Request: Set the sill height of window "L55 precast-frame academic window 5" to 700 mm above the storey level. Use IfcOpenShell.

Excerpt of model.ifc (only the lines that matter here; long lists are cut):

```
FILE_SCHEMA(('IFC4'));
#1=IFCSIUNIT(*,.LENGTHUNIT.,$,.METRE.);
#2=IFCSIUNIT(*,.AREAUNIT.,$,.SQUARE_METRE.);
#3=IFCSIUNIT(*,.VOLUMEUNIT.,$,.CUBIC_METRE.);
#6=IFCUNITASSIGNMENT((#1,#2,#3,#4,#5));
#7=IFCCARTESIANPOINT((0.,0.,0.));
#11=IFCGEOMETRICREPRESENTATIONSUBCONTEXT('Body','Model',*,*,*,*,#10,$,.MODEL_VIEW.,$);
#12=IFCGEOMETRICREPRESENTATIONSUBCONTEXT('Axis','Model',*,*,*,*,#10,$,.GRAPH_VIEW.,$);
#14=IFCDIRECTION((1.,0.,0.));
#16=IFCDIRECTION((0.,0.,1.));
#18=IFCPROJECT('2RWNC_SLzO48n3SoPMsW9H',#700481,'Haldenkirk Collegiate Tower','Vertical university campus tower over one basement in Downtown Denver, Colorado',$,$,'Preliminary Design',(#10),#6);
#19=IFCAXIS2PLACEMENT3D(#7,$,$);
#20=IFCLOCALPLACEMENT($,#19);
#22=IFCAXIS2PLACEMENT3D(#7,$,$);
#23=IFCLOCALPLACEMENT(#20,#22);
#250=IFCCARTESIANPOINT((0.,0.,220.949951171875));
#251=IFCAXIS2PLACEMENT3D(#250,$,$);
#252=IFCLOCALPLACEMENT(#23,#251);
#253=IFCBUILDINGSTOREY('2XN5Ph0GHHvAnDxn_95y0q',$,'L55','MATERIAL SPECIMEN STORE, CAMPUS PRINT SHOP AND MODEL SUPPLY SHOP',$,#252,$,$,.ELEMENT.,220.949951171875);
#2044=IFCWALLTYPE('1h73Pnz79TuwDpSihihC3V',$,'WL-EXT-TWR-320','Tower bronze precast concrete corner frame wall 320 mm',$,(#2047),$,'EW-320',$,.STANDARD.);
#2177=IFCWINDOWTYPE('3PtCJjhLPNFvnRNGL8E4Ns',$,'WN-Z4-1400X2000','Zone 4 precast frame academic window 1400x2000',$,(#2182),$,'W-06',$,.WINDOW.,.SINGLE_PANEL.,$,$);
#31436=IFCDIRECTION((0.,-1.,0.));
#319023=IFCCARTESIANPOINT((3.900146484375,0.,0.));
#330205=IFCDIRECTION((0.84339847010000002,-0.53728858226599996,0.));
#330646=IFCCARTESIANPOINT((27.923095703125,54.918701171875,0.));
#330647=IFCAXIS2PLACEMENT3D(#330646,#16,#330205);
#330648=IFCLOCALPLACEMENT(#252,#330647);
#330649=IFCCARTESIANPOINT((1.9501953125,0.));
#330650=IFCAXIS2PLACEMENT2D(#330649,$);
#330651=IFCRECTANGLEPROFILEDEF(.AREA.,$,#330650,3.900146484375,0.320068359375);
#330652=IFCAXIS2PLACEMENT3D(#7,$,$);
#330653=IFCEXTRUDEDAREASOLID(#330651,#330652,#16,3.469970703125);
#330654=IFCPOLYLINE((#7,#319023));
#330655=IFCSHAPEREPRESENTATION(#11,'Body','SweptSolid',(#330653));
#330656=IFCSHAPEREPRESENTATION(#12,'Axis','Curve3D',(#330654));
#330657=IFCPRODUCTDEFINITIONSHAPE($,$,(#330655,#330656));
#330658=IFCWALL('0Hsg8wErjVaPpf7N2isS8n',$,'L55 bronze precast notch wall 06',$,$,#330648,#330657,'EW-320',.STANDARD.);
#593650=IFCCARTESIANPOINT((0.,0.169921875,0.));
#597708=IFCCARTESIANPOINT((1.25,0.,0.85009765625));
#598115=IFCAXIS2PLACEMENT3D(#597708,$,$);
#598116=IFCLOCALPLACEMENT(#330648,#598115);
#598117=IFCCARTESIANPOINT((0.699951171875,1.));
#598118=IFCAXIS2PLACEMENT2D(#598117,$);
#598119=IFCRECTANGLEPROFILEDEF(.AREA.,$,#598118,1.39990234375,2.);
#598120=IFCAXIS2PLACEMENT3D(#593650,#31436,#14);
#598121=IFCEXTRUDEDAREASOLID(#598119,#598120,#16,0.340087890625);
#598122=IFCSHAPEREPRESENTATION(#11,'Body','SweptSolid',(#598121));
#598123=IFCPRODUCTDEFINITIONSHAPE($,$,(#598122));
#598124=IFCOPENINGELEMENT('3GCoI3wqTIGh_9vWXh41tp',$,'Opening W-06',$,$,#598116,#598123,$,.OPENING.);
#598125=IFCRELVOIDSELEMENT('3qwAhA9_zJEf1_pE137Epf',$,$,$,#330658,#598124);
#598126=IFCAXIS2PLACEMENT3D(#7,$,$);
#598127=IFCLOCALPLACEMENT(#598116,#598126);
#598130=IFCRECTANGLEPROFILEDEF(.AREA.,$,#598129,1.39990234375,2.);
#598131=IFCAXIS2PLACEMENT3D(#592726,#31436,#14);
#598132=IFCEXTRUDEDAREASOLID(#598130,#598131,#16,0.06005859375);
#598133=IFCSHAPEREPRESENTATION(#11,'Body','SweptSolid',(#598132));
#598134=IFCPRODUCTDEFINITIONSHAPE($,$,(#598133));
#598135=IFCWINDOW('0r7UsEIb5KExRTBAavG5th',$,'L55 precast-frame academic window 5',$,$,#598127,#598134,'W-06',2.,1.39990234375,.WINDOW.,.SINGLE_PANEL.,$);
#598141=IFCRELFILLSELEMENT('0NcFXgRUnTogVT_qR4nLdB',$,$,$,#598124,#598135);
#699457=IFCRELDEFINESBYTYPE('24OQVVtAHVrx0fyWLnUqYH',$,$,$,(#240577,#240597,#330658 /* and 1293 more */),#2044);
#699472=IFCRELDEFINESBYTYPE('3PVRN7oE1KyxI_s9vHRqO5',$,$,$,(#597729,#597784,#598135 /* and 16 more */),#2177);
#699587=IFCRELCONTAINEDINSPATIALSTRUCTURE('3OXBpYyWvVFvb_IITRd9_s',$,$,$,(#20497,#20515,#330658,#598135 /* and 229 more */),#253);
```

```python
import numpy as np
import ifcopenshell
import ifcopenshell.api.geometry
import ifcopenshell.geom
import ifcopenshell.util.element
import ifcopenshell.util.placement
import ifcopenshell.util.shape
import ifcopenshell.util.unit

model = ifcopenshell.open("model.ifc")
unit_scale = ifcopenshell.util.unit.calculate_unit_scale(model)

window = model.by_id(598135)
opening = window.FillsVoids[0].RelatingOpeningElement
storey = ifcopenshell.util.element.get_container(window, ifc_class="IfcBuildingStorey")
level = ifcopenshell.util.placement.get_local_placement(storey.ObjectPlacement)[2, 3]

# The opening's origin need not be at the sill, so measure its lowest point.
shape = ifcopenshell.geom.create_shape(ifcopenshell.geom.settings(), opening)
bottom = ifcopenshell.util.shape.get_shape_bottom_elevation(shape, shape.geometry) / unit_scale
dz = level + 0.7 - bottom

shift = np.array([0.0, 0.0, dz])
# The window is placed relative to its opening, so it follows when the opening moves.
matrix = ifcopenshell.util.placement.get_local_placement(opening.ObjectPlacement)
matrix[:3, 3] += shift
ifcopenshell.api.geometry.edit_object_placement(
    model, product=opening, matrix=matrix, is_si=False, should_transform_children=True
)

print(f"moved by {dz * unit_scale:+.3f} m")

model.write("model_rev.ifc")
```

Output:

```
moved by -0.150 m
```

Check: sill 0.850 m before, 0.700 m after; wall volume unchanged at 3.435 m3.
